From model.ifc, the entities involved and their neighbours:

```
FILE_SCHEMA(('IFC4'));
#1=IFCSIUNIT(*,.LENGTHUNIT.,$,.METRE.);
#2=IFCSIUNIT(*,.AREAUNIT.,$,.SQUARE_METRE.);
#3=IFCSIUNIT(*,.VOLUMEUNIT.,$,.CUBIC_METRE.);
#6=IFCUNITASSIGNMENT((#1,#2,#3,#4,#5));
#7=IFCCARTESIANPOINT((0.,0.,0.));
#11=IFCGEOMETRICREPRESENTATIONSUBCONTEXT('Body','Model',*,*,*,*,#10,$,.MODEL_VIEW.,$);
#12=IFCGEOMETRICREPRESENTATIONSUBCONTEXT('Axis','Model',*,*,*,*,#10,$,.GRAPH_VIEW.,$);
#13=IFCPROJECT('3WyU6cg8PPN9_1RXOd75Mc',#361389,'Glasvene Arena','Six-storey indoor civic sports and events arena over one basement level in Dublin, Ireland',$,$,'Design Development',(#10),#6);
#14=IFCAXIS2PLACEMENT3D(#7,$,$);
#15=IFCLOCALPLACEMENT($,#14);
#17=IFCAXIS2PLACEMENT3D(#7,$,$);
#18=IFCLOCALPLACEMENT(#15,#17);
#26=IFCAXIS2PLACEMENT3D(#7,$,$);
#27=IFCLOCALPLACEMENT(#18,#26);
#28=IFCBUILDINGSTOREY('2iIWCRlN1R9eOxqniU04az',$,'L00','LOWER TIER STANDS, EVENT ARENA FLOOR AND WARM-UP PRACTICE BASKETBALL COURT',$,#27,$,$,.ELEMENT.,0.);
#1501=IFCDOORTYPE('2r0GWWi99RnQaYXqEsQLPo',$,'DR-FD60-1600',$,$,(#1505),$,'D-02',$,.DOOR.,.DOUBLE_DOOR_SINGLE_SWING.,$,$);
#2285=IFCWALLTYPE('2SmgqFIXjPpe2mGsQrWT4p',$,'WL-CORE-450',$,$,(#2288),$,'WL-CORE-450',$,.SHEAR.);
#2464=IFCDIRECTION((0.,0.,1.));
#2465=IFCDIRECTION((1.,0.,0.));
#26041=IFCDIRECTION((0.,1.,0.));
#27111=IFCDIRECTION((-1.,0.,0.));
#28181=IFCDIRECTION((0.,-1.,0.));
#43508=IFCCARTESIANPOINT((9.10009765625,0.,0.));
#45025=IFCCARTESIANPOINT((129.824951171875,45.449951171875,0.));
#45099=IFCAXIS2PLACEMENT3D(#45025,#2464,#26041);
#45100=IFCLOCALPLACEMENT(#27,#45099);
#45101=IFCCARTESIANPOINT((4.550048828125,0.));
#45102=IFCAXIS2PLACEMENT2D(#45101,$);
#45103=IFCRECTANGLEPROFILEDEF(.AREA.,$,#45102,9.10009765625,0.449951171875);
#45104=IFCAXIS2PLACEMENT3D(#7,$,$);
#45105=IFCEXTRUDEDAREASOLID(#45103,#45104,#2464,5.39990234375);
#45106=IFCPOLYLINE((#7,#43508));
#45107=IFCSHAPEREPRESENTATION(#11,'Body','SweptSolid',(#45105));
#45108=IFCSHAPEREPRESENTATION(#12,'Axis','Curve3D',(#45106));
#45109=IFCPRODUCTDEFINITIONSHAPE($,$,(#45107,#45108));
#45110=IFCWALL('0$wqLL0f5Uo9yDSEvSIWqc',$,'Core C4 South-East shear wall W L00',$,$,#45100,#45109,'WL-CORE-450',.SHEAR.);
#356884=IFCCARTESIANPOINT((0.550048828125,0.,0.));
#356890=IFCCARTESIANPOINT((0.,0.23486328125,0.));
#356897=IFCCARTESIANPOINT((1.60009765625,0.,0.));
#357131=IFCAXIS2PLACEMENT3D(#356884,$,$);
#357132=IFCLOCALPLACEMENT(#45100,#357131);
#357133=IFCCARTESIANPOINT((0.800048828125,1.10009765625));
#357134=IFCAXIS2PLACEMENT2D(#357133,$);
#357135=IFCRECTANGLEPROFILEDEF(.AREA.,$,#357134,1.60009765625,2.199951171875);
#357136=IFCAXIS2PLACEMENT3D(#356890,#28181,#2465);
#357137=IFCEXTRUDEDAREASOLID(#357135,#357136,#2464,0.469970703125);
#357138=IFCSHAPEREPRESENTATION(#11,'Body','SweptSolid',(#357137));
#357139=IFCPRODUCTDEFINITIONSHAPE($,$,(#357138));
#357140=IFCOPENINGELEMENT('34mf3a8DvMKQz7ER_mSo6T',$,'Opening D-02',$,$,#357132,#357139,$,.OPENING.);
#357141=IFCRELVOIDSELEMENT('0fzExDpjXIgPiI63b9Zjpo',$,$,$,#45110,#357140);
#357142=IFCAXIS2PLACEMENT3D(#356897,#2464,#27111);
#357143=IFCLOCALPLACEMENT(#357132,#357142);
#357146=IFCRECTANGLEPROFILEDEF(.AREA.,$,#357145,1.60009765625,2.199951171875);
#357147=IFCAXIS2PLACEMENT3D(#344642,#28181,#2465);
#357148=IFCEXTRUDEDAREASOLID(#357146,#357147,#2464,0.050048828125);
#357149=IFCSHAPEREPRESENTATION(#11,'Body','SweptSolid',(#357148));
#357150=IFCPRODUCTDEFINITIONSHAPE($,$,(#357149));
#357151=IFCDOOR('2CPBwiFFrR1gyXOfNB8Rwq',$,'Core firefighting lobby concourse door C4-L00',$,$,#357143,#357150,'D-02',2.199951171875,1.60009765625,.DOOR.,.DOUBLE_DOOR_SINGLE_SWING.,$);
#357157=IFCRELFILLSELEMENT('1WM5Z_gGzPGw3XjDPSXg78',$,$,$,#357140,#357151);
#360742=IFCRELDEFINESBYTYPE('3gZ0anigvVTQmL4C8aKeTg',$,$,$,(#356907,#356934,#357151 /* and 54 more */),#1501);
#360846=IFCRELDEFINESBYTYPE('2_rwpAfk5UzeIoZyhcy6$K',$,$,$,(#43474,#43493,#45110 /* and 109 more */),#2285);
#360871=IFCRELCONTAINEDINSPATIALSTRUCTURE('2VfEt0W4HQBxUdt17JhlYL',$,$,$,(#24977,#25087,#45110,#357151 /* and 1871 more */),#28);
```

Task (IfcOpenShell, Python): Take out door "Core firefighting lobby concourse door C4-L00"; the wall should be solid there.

```python
import ifcopenshell
import ifcopenshell.api.feature
import ifcopenshell.api.root
import ifcopenshell.geom
import ifcopenshell.util.shape

model = ifcopenshell.open("model.ifc")
settings = ifcopenshell.geom.settings()


def volume(element):
    """Net volume in cubic metres, openings subtracted."""
    shape = ifcopenshell.geom.create_shape(settings, element)
    return ifcopenshell.util.shape.get_volume(shape.geometry)


door = model.by_id(357151)
opening = door.FillsVoids[0].RelatingOpeningElement
wall = opening.VoidsElements[0].RelatingBuildingElement
before = volume(wall)

ifcopenshell.api.root.remove_product(model, product=door)
ifcopenshell.api.feature.remove_feature(model, feature=opening)

after = volume(wall)

print(f"wall volume {before:.3f} -> {after:.3f} m3")

model.write("model_edited.ifc")
```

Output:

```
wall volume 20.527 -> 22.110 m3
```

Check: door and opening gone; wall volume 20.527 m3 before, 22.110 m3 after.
